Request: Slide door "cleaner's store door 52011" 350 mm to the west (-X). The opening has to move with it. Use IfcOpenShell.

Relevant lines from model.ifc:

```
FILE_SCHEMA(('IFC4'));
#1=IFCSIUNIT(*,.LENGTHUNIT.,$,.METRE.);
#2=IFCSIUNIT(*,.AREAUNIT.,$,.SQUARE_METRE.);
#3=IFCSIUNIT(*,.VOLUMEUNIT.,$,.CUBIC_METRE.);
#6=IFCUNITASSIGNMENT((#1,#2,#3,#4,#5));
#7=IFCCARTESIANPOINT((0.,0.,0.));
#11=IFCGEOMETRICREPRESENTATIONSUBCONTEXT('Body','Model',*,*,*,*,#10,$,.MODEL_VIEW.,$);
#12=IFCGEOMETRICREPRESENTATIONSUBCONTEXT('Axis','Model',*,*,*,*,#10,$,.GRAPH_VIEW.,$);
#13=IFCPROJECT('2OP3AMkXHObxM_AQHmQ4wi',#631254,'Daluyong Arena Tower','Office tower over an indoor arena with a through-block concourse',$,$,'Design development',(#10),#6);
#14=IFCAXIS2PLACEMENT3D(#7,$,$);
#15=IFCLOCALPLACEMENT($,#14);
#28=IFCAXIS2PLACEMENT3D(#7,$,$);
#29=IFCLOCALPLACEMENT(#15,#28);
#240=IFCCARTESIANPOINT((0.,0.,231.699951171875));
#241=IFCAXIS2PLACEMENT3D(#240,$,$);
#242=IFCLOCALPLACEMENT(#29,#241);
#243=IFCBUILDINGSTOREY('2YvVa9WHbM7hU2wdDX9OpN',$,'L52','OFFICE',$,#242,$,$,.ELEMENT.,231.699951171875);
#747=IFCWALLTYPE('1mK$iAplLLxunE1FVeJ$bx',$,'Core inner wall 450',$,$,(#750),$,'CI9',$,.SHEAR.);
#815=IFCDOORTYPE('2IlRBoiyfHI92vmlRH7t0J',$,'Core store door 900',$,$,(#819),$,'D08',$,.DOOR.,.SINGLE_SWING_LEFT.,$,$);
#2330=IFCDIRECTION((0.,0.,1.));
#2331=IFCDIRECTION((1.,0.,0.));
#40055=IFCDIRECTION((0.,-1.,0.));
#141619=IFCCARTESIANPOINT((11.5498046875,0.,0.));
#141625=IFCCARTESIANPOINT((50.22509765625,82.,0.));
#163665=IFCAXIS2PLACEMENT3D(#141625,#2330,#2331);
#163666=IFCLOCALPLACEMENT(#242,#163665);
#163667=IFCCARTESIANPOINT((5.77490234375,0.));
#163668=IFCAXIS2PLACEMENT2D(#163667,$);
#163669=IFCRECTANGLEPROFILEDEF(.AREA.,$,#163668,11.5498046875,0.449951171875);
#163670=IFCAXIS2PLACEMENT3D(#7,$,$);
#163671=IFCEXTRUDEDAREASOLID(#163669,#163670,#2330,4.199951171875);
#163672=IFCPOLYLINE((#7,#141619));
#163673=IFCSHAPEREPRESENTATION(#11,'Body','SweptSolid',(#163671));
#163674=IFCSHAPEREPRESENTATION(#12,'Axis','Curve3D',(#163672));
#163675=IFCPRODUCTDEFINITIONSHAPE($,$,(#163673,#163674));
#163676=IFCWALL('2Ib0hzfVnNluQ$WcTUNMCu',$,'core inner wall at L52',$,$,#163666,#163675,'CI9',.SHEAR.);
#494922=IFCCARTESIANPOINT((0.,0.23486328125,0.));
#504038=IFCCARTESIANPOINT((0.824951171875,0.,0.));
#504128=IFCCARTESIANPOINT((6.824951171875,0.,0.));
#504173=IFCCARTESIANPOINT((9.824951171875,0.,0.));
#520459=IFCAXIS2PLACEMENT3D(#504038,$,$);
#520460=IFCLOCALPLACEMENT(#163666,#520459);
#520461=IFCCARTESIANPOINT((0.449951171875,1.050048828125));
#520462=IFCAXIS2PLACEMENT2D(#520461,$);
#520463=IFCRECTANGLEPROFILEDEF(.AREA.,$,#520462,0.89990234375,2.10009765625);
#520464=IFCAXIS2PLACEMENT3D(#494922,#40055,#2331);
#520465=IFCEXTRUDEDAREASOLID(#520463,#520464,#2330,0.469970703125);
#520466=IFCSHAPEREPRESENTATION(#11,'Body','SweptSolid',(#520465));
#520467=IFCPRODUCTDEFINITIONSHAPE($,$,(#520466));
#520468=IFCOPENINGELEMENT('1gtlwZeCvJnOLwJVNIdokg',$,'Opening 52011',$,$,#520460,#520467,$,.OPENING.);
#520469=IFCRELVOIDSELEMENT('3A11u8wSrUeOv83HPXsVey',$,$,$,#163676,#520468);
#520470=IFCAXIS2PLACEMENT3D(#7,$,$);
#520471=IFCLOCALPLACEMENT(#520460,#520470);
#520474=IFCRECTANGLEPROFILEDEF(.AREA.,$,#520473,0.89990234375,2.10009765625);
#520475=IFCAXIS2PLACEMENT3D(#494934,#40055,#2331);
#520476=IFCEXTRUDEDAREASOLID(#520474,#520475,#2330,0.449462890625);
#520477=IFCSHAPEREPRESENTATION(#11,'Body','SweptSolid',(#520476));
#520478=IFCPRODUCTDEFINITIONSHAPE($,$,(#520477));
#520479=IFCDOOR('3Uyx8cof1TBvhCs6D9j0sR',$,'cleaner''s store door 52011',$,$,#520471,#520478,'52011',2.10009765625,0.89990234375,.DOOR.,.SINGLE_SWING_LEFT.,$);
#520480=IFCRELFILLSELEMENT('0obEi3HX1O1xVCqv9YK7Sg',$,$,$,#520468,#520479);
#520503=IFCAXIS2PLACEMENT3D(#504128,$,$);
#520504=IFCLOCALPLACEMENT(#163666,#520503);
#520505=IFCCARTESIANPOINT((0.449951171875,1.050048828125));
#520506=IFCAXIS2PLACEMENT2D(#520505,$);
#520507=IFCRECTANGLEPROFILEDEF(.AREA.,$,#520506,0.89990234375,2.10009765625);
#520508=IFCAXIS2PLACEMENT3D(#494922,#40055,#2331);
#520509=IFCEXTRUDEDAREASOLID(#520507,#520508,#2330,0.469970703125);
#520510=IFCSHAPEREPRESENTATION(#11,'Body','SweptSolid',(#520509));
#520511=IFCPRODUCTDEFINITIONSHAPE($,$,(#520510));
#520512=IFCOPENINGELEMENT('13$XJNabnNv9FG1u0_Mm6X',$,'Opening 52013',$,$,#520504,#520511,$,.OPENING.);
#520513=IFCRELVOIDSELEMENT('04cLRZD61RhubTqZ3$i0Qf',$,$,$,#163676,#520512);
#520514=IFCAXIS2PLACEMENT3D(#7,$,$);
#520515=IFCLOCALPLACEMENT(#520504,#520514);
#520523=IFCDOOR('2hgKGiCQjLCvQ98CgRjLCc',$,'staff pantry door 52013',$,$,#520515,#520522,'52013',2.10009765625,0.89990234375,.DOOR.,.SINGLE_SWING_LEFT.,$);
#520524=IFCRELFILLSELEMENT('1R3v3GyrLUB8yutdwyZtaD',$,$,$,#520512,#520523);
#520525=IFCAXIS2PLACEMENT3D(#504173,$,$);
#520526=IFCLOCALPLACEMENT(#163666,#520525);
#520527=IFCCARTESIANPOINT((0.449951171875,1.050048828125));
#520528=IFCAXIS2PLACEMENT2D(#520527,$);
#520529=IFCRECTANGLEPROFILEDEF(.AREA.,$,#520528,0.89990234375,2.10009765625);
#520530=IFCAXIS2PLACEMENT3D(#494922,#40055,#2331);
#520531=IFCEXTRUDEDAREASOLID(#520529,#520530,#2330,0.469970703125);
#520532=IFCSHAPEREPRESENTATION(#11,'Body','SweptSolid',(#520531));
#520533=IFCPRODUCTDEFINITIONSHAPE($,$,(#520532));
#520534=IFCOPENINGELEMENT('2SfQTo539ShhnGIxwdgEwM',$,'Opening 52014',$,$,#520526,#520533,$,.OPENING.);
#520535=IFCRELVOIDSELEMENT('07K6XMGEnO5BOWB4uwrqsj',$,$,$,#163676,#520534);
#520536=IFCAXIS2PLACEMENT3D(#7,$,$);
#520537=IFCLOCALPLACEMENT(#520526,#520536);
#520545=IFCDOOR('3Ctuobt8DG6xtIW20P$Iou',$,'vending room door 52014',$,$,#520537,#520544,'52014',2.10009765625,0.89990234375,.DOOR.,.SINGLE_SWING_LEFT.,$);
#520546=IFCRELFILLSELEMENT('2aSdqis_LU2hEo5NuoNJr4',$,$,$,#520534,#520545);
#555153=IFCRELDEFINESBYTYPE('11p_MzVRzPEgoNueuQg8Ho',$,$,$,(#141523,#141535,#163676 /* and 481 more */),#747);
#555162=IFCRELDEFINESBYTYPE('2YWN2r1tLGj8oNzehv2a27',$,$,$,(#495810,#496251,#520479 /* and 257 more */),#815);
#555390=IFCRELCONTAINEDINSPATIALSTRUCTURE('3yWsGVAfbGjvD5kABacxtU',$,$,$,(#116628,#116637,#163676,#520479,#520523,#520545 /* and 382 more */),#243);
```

```python
import ifcopenshell
import ifcopenshell.api.geometry
import ifcopenshell.util.placement
import ifcopenshell.util.unit

model = ifcopenshell.open("model.ifc")
unit_scale = ifcopenshell.util.unit.calculate_unit_scale(model)

door = model.by_id(520479)
opening = door.FillsVoids[0].RelatingOpeningElement
wall = opening.VoidsElements[0].RelatingBuildingElement

wall_matrix = ifcopenshell.util.placement.get_local_placement(wall.ObjectPlacement)
shift = wall_matrix[:3, 0] * -0.35 / unit_scale
before = ifcopenshell.util.placement.get_local_placement(door.ObjectPlacement)[:3, 3].copy()

# The door is placed relative to its opening, so it follows when the opening moves.
matrix = ifcopenshell.util.placement.get_local_placement(opening.ObjectPlacement)
matrix[:3, 3] += shift
ifcopenshell.api.geometry.edit_object_placement(
    model, product=opening, matrix=matrix, is_si=False, should_transform_children=True
)

after = ifcopenshell.util.placement.get_local_placement(door.ObjectPlacement)[:3, 3]
print("door moved by", (after - before).round(3) + 0.0)

model.write("model_rev.ifc")
```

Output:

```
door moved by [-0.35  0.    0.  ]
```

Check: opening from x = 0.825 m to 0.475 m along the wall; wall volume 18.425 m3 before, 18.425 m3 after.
